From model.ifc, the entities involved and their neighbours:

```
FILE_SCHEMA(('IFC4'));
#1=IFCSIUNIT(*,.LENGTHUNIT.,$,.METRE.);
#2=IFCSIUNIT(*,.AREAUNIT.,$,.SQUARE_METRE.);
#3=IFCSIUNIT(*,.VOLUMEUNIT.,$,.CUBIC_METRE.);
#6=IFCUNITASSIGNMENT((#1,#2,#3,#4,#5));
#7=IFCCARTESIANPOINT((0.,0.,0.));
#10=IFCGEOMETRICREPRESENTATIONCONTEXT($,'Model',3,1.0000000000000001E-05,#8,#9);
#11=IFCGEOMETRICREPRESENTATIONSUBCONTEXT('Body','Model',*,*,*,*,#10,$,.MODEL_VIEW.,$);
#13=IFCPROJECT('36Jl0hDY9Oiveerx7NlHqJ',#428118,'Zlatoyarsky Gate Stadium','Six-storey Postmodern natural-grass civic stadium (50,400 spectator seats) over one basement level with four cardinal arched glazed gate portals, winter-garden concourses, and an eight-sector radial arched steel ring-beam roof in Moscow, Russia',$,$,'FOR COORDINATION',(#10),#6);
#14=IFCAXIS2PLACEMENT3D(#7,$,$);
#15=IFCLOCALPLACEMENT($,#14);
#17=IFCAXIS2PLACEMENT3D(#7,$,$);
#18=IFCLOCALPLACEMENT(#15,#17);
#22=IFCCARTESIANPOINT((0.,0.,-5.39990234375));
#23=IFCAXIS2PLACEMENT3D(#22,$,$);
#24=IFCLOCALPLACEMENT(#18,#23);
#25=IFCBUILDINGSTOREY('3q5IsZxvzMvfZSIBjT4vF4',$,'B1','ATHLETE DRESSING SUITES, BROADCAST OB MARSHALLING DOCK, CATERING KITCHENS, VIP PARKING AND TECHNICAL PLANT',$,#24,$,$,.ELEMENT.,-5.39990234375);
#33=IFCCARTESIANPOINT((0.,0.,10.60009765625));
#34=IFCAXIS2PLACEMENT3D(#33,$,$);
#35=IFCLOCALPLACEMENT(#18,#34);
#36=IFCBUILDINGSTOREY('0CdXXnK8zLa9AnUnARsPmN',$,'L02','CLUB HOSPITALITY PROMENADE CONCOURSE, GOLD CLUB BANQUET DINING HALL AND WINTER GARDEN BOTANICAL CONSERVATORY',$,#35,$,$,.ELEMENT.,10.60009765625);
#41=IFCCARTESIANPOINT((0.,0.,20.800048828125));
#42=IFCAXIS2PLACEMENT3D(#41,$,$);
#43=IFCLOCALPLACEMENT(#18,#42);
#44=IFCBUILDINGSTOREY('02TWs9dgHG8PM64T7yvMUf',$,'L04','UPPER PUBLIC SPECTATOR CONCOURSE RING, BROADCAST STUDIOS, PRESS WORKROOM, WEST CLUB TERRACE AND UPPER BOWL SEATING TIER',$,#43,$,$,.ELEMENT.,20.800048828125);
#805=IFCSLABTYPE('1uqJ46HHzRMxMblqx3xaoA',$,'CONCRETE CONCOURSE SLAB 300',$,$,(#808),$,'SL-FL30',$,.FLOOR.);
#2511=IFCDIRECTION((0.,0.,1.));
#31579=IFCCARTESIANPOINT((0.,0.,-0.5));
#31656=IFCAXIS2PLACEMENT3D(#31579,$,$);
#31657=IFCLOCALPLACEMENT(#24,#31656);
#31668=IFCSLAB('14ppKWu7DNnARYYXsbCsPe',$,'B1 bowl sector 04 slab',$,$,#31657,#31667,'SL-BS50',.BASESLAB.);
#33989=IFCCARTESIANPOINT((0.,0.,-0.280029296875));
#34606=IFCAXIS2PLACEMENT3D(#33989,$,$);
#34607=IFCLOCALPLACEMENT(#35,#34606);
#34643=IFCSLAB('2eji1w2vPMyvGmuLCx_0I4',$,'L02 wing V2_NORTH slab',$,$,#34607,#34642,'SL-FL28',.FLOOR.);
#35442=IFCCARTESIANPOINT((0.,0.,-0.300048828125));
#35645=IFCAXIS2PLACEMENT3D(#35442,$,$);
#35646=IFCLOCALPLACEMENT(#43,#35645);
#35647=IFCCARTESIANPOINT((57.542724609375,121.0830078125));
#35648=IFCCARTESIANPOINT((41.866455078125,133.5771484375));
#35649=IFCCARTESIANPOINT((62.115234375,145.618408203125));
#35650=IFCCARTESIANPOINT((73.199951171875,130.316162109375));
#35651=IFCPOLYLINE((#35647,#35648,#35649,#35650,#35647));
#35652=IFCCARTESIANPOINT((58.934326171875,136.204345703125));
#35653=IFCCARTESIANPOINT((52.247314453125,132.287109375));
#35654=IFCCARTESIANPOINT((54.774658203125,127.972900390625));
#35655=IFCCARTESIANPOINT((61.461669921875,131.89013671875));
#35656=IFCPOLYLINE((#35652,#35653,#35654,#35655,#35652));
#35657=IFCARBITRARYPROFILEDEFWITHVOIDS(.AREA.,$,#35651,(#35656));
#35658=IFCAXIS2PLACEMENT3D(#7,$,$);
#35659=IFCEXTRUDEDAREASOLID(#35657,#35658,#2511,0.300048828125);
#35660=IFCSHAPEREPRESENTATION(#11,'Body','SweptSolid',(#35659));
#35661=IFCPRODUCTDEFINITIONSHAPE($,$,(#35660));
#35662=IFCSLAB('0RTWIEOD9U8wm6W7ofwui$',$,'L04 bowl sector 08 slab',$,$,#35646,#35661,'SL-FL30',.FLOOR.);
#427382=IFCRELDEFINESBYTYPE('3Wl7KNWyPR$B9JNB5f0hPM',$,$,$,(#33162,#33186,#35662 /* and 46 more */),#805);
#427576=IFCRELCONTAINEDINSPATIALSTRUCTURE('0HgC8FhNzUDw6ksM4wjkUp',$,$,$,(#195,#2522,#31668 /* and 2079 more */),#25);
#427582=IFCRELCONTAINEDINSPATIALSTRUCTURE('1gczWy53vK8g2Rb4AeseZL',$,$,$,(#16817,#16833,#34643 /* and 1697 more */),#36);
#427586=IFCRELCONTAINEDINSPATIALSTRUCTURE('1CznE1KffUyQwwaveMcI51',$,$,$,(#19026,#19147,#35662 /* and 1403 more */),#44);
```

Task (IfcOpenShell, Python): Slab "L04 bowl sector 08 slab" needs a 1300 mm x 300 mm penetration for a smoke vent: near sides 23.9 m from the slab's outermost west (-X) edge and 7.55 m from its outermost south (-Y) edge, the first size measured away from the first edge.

```python
import numpy as np
import ifcopenshell
import ifcopenshell.api.feature
import ifcopenshell.api.geometry
import ifcopenshell.api.root
import ifcopenshell.geom
import ifcopenshell.util.placement
import ifcopenshell.util.representation
import ifcopenshell.util.shape
import ifcopenshell.util.unit

model = ifcopenshell.open("model.ifc")
unit_scale = ifcopenshell.util.unit.calculate_unit_scale(model)
settings = ifcopenshell.geom.settings()


def volume(element):
    """Net volume in cubic metres, openings subtracted."""
    shape = ifcopenshell.geom.create_shape(settings, element)
    return ifcopenshell.util.shape.get_volume(shape.geometry)


slab = model.by_guid("0RTWIEOD9U8wm6W7ofwui$")
before = volume(slab)

# Extent in the slab's own axes, in metres. The edges named are its -X and -Y sides.
slab_shape = ifcopenshell.geom.create_shape(settings, slab)
vertices = ifcopenshell.util.shape.get_vertices(slab_shape.geometry)
x_min, y_min, bottom = vertices.min(axis=0)
top = vertices[:, 2].max()

opening = ifcopenshell.api.root.create_entity(model, ifc_class="IfcOpeningElement", name="Smoke vent opening", predefined_type="OPENING")
context = ifcopenshell.util.representation.get_context(model, "Model", "Body", "MODEL_VIEW")
width, depth = 1.3, 0.3
outline = [(0.0, 0.0), (width, 0.0), (width, depth), (0.0, depth), (0.0, 0.0)]
# Overshoot both faces by 50 mm so the cut is clean.
shape = ifcopenshell.api.geometry.add_slab_representation(
    model, context=context, depth=top - bottom + 0.1, polyline=outline
)
ifcopenshell.api.geometry.assign_representation(model, product=opening, representation=shape)

matrix = ifcopenshell.util.placement.get_local_placement(slab.ObjectPlacement)
matrix[:, 3] = matrix @ np.append(np.array([x_min + 23.9, y_min + 7.55, bottom - 0.05]) / unit_scale, 1.0)
ifcopenshell.api.geometry.edit_object_placement(model, product=opening, matrix=matrix, is_si=False)
ifcopenshell.api.feature.add_feature(model, feature=opening, element=slab)

after = volume(slab)

print(f"slab volume {before:.3f} -> {after:.3f} m3")

model.write("model_v2.ifc")
```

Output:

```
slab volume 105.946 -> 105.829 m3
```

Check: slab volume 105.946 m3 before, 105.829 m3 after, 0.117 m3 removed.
